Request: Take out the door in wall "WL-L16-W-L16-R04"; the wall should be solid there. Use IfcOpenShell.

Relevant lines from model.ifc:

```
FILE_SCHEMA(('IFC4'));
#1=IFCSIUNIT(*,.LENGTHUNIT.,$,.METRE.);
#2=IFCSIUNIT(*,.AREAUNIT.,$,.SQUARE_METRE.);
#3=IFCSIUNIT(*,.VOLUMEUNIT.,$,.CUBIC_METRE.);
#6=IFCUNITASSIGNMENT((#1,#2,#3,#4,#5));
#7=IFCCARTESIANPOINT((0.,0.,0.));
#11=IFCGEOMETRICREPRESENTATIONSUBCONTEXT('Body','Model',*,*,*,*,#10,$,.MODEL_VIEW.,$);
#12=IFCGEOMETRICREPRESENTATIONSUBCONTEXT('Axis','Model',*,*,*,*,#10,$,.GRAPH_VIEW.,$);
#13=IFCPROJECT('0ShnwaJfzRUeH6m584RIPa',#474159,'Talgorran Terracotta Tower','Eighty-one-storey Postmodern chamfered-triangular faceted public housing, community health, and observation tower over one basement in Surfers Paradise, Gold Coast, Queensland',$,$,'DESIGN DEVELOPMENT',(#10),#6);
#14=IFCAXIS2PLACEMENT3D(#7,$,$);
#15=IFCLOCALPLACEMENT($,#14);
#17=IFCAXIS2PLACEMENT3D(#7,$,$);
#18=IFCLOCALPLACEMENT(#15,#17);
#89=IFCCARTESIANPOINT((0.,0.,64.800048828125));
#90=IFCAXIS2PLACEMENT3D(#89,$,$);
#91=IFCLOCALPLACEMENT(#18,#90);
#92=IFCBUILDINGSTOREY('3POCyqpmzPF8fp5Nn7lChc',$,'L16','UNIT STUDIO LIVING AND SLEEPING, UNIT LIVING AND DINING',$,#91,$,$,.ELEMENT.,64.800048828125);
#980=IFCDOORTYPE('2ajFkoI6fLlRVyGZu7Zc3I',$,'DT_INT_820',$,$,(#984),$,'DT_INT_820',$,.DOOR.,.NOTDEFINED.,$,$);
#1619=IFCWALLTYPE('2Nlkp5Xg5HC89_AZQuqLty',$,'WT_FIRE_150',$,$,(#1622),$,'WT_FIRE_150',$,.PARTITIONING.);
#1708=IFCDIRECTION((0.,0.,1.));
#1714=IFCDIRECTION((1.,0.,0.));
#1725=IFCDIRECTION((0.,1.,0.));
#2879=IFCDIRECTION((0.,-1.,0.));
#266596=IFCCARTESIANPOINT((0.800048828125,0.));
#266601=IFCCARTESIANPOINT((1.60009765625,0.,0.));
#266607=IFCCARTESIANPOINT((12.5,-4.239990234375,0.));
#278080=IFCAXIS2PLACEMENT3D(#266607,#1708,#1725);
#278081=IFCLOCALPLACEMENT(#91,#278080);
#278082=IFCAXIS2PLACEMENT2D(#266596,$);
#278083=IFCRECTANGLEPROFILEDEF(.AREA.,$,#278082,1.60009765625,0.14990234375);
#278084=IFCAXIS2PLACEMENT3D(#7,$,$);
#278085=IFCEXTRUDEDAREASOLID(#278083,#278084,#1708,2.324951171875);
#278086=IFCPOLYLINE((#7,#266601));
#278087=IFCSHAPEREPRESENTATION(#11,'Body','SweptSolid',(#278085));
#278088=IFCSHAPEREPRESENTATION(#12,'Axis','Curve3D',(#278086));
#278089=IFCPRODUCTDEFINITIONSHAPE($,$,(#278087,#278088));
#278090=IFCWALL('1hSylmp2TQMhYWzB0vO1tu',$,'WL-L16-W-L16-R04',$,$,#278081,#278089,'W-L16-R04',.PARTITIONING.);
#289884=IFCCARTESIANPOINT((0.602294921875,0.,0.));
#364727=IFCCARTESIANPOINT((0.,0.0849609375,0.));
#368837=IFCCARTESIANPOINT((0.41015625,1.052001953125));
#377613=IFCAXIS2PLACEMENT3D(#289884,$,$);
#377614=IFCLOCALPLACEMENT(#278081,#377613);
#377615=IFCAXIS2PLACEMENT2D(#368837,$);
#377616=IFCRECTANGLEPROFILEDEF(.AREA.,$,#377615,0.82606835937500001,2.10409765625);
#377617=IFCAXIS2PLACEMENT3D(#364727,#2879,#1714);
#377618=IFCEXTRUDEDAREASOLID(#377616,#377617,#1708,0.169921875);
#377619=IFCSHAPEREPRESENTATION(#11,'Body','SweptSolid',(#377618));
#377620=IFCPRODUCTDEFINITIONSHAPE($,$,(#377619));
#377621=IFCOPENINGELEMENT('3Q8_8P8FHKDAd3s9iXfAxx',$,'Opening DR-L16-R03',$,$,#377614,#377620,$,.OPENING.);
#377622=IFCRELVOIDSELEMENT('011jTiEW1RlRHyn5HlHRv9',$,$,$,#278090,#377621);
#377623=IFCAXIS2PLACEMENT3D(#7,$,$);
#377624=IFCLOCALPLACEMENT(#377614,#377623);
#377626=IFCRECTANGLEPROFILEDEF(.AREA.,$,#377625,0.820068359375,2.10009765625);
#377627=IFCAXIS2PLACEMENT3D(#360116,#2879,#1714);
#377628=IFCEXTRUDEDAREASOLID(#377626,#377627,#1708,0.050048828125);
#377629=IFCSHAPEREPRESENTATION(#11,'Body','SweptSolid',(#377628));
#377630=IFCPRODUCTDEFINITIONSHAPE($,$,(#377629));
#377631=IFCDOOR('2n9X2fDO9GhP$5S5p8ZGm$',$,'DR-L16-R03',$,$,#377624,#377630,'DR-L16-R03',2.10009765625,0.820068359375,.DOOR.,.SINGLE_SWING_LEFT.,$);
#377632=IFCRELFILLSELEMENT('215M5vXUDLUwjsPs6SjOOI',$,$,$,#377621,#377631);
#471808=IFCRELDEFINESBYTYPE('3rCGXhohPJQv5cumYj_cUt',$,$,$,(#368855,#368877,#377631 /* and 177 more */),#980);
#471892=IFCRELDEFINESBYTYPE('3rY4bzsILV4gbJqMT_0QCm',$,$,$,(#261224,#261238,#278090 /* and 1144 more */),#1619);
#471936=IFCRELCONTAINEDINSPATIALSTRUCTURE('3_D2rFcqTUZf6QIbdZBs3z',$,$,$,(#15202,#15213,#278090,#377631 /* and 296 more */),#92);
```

```python
import ifcopenshell
import ifcopenshell.api.feature
import ifcopenshell.api.root
import ifcopenshell.geom
import ifcopenshell.util.shape

model = ifcopenshell.open("model.ifc")
settings = ifcopenshell.geom.settings()


def volume(element):
    """Net volume in cubic metres, openings subtracted."""
    shape = ifcopenshell.geom.create_shape(settings, element)
    return ifcopenshell.util.shape.get_volume(shape.geometry)


door = model.by_id(377631)
opening = door.FillsVoids[0].RelatingOpeningElement
wall = opening.VoidsElements[0].RelatingBuildingElement
before = volume(wall)

ifcopenshell.api.root.remove_product(model, product=door)
ifcopenshell.api.feature.remove_feature(model, feature=opening)

after = volume(wall)

print(f"wall volume {before:.3f} -> {after:.3f} m3")

model.write("model_updated.ifc")
```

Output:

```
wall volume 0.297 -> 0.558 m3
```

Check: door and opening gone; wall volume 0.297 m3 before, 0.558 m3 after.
